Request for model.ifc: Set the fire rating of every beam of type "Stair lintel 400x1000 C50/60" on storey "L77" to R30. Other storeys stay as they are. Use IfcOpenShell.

First a look at what the model holds.

```python
import ifcopenshell
import ifcopenshell.util.element

model = ifcopenshell.open("model.ifc")
print(model.schema)
storey = next(s for s in model.by_type("IfcBuildingStorey") if s.Name == "L77")
beams = [e for e in ifcopenshell.util.element.get_decomposition(storey) if e.is_a("IfcBeam")]
seen = {}
for e in beams:
    element_type = ifcopenshell.util.element.get_type(e)
    key = (element_type.Name if element_type != e and element_type else None, ifcopenshell.util.element.get_pset(e, "Pset_BeamCommon", "FireRating"))
    seen[key] = seen.get(key, 0) + 1
for (name, value), count in sorted(seen.items(), key=str):
    print(count, "x", name, "|", value)
```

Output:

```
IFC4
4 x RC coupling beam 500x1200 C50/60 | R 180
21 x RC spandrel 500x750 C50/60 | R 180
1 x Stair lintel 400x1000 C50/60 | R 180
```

```python
import ifcopenshell
import ifcopenshell.api.pset
import ifcopenshell.util.element

model = ifcopenshell.open("model.ifc")

storey = next(s for s in model.by_type("IfcBuildingStorey") if s.Name == "L77")
beams = [e for e in ifcopenshell.util.element.get_decomposition(storey) if e.is_a("IfcBeam")]

count = 0
for e in beams:
    element_type = ifcopenshell.util.element.get_type(e)
    if element_type in (None, e) or element_type.Name != "Stair lintel 400x1000 C50/60":
        continue
    found = ifcopenshell.util.element.get_pset(e, "Pset_BeamCommon", should_inherit=False)
    if found:
        pset = model.by_id(found["id"])
        if len(ifcopenshell.util.element.get_elements_by_pset(pset)) > 1:
            pset = ifcopenshell.api.pset.unshare_pset(model, products=[e], pset=pset)[0]
    else:
        pset = ifcopenshell.api.pset.add_pset(model, product=e, name="Pset_BeamCommon")
    ifcopenshell.api.pset.edit_pset(model, pset=pset, properties={"FireRating": "R30"})
    count += 1

print(count, "beams updated")

model.write("model-out.ifc")
```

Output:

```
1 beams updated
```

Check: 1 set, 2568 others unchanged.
